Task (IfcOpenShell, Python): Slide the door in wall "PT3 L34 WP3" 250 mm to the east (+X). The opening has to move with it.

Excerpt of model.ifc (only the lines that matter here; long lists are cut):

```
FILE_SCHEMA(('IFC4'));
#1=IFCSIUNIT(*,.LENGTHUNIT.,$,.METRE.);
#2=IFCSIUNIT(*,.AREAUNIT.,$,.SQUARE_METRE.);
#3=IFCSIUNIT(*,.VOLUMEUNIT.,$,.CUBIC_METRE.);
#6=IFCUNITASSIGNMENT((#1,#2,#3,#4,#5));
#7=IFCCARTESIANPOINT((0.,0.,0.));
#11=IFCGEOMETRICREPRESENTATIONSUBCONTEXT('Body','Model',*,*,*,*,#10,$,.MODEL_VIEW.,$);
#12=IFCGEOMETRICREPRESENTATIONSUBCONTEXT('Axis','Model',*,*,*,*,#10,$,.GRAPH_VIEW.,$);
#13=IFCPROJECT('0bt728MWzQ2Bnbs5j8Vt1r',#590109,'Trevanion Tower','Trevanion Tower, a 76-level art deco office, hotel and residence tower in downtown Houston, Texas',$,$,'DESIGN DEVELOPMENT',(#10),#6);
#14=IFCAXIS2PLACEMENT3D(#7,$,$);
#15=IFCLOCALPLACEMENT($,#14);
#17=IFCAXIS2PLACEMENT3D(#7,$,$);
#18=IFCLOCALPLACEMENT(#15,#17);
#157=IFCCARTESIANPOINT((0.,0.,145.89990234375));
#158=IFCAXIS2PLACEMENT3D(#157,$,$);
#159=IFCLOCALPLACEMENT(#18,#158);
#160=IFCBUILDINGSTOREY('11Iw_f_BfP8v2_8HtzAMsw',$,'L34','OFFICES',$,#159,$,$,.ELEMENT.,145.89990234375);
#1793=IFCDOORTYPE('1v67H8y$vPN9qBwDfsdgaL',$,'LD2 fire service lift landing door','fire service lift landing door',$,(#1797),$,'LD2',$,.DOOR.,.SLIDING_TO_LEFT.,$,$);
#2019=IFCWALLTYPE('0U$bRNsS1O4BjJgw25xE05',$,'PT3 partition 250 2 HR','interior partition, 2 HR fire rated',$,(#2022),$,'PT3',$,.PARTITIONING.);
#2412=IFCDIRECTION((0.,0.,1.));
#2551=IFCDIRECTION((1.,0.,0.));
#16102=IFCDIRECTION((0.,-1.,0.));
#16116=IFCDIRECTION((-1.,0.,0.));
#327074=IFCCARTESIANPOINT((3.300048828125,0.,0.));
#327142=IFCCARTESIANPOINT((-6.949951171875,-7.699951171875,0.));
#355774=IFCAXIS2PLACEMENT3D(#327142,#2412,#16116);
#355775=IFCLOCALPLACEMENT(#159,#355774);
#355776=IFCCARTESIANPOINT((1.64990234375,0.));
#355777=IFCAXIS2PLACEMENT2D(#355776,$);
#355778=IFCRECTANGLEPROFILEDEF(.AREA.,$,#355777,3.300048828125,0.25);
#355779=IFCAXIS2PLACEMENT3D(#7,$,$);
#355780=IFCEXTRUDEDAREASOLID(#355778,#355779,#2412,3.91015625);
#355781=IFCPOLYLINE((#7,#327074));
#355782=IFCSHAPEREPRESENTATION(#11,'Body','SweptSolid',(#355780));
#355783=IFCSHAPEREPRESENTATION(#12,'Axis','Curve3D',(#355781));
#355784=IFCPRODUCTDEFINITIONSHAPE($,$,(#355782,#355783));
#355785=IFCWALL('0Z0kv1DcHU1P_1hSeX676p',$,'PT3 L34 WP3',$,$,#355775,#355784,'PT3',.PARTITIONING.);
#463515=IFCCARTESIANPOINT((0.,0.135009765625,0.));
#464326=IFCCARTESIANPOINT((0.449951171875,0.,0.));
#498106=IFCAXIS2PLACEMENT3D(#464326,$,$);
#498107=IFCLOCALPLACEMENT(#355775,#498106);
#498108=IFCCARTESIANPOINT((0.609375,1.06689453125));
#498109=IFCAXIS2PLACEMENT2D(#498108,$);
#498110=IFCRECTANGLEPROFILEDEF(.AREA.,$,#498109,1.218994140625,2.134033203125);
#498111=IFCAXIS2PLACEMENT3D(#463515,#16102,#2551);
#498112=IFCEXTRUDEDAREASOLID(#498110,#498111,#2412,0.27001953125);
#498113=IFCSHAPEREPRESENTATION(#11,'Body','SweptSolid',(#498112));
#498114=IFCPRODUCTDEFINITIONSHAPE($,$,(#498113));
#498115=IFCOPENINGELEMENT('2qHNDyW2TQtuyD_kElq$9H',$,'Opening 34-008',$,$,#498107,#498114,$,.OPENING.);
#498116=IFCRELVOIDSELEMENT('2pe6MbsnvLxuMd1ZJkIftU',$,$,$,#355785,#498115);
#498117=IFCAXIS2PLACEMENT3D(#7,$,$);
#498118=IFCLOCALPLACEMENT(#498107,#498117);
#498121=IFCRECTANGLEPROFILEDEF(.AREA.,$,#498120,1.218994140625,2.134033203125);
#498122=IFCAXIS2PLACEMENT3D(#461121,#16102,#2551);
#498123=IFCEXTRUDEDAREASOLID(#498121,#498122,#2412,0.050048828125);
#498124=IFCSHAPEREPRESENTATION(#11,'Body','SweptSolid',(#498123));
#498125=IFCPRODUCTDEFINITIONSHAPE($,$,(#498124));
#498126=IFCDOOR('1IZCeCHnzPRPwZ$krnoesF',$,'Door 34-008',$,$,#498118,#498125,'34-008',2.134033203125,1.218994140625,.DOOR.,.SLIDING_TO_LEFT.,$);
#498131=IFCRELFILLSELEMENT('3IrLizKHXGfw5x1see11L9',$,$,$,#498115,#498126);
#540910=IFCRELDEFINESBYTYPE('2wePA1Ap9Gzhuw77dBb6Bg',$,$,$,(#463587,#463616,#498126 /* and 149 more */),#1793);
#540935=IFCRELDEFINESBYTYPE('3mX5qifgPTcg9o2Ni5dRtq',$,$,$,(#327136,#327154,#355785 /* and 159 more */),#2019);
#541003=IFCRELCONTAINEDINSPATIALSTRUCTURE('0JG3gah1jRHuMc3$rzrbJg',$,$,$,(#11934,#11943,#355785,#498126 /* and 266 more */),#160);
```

```python
import ifcopenshell
import ifcopenshell.api.geometry
import ifcopenshell.util.placement
import ifcopenshell.util.unit

model = ifcopenshell.open("model.ifc")
unit_scale = ifcopenshell.util.unit.calculate_unit_scale(model)

door = model.by_guid("1IZCeCHnzPRPwZ$krnoesF")
opening = door.FillsVoids[0].RelatingOpeningElement
wall = opening.VoidsElements[0].RelatingBuildingElement

wall_matrix = ifcopenshell.util.placement.get_local_placement(wall.ObjectPlacement)
shift = wall_matrix[:3, 0] * -0.25 / unit_scale
before = ifcopenshell.util.placement.get_local_placement(door.ObjectPlacement)[:3, 3].copy()

# The door is placed relative to its opening, so it follows when the opening moves.
matrix = ifcopenshell.util.placement.get_local_placement(opening.ObjectPlacement)
matrix[:3, 3] += shift
ifcopenshell.api.geometry.edit_object_placement(
    model, product=opening, matrix=matrix, is_si=False, should_transform_children=True
)

after = ifcopenshell.util.placement.get_local_placement(door.ObjectPlacement)[:3, 3]
print("door moved by", (after - before).round(3) + 0.0)

model.write("model-out.ifc")
```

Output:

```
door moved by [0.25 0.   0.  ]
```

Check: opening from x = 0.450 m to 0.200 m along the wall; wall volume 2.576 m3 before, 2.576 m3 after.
